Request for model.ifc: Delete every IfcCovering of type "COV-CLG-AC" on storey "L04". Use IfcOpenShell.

First a look at what the model holds.

```python
import ifcopenshell
import ifcopenshell.util.element

model = ifcopenshell.open("model.ifc")
print(model.schema)
storey = next(s for s in model.by_type("IfcBuildingStorey") if s.Name == "L04")
coverings = [e for e in ifcopenshell.util.element.get_decomposition(storey) if e.is_a("IfcCovering")]
seen = {}
for e in coverings:
    element_type = ifcopenshell.util.element.get_type(e)
    name = element_type.Name if element_type not in (None, e) else None
    seen[name] = seen.get(name, 0) + 1
for name, count in sorted(seen.items(), key=str):
    print(count, "x", name)
```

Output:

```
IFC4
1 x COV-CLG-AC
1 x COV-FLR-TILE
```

```python
import ifcopenshell
import ifcopenshell.api.root
import ifcopenshell.util.element

model = ifcopenshell.open("model.ifc")

storey = next(s for s in model.by_type("IfcBuildingStorey") if s.Name == "L04")
coverings = [e for e in ifcopenshell.util.element.get_decomposition(storey) if e.is_a("IfcCovering")]
targets = [e for e in coverings if (t := ifcopenshell.util.element.get_type(e)) not in (None, e) and t.Name == "COV-CLG-AC"]

for e in targets:
    ifcopenshell.api.root.remove_product(model, product=e)
print(len(targets), "removed")

model.write("model_rev.ifc")
```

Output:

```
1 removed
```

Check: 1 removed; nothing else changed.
